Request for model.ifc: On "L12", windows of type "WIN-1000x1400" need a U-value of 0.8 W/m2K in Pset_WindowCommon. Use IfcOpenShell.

First a look at what the model holds.

```python
import ifcopenshell
import ifcopenshell.util.element

model = ifcopenshell.open("model.ifc")
print(model.schema)
storey = next(s for s in model.by_type("IfcBuildingStorey") if s.Name == "L12")
windows = [e for e in ifcopenshell.util.element.get_decomposition(storey) if e.is_a("IfcWindow")]
seen = {}
for e in windows:
    element_type = ifcopenshell.util.element.get_type(e)
    key = (element_type.Name if element_type != e and element_type else None, ifcopenshell.util.element.get_pset(e, "Pset_WindowCommon", "ThermalTransmittance"))
    seen[key] = seen.get(key, 0) + 1
for (name, value), count in sorted(seen.items(), key=str):
    print(count, "x", name, "|", value)
```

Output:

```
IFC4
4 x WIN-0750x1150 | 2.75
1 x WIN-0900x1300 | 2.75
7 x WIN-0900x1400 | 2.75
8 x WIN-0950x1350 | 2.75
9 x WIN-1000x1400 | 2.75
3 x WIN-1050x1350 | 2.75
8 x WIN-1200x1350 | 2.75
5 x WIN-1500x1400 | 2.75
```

```python
import ifcopenshell
import ifcopenshell.api.pset
import ifcopenshell.util.element

model = ifcopenshell.open("model.ifc")

storey = next(s for s in model.by_type("IfcBuildingStorey") if s.Name == "L12")
windows = [e for e in ifcopenshell.util.element.get_decomposition(storey) if e.is_a("IfcWindow")]

count = 0
for e in windows:
    element_type = ifcopenshell.util.element.get_type(e)
    if element_type in (None, e) or element_type.Name != "WIN-1000x1400":
        continue
    # add_pset returns the element's existing set when there is one.
    pset = ifcopenshell.api.pset.add_pset(model, product=e, name="Pset_WindowCommon")
    ifcopenshell.api.pset.edit_pset(model, pset=pset, properties={"ThermalTransmittance": 0.8})
    count += 1

print(count, "windows updated")

model.write("model_v2.ifc")
```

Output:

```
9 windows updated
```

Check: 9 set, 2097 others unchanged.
